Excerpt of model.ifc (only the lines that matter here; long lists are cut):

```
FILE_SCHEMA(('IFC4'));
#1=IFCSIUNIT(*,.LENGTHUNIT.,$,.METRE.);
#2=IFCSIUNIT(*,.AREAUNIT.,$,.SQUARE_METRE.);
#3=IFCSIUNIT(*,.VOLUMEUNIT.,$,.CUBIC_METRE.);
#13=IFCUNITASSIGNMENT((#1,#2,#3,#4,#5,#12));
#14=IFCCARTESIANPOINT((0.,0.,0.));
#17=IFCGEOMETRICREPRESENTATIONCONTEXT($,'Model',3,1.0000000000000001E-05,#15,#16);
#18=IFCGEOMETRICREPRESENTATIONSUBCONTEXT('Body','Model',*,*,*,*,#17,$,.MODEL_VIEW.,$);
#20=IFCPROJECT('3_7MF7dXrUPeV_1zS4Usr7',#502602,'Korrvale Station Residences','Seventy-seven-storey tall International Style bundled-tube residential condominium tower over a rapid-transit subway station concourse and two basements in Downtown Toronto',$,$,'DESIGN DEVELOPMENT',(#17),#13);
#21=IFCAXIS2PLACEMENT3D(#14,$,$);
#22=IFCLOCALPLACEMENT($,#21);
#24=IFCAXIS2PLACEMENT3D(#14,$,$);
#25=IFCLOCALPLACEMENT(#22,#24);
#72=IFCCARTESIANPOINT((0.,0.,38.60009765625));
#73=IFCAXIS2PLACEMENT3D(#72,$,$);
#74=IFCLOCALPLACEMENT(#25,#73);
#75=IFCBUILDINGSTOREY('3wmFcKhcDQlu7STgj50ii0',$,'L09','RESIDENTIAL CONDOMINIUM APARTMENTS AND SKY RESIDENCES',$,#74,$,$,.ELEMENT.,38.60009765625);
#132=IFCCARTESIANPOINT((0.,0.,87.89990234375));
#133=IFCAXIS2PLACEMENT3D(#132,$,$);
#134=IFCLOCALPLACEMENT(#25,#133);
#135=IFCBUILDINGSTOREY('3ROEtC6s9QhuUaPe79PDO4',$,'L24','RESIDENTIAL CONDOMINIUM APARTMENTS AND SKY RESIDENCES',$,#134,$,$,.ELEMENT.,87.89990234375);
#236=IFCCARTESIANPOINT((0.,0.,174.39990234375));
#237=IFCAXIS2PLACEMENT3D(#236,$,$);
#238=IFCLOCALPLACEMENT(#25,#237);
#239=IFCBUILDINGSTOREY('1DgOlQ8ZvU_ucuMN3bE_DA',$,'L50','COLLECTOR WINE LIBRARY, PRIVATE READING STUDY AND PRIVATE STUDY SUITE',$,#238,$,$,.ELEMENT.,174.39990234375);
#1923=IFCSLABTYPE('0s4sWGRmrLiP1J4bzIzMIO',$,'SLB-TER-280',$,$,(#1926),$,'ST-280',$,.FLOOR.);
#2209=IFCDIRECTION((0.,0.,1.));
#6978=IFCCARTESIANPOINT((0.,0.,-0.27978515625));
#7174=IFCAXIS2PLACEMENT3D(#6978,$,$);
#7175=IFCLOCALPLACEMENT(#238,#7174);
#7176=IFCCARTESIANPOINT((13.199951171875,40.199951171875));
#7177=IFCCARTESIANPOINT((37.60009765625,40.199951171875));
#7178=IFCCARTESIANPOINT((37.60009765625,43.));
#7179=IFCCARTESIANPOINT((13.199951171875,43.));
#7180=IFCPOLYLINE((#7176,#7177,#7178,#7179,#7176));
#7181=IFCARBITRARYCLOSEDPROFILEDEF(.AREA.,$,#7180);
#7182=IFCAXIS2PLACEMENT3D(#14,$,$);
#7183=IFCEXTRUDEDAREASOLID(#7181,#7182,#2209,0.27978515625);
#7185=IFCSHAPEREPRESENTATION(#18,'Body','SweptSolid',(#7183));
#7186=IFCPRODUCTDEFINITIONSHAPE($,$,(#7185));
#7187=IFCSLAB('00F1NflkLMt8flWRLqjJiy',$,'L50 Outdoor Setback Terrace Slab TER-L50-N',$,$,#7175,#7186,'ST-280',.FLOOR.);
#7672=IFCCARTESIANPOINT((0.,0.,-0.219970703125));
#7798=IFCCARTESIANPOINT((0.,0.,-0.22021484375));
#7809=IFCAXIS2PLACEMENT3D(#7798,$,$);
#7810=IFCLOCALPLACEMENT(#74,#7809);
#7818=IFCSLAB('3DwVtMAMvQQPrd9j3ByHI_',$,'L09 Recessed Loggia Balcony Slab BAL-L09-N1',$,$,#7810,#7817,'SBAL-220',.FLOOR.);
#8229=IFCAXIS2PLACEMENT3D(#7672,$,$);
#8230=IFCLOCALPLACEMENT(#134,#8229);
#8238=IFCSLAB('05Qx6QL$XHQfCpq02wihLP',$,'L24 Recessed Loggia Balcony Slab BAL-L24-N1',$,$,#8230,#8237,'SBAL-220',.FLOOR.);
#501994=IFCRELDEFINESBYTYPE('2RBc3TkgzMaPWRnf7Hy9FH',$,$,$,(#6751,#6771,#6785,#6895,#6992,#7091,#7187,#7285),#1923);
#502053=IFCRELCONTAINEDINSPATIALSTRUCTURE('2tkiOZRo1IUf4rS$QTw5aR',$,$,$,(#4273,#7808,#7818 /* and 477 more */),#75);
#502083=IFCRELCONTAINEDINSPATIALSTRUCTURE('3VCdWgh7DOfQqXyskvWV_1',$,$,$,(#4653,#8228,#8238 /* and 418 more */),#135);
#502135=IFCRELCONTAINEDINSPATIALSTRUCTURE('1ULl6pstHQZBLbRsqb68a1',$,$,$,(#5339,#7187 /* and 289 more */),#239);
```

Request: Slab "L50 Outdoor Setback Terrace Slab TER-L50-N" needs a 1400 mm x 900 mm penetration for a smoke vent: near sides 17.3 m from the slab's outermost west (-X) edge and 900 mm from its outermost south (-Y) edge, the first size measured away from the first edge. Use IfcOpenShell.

```python
import numpy as np
import ifcopenshell
import ifcopenshell.api.feature
import ifcopenshell.api.geometry
import ifcopenshell.api.root
import ifcopenshell.geom
import ifcopenshell.util.placement
import ifcopenshell.util.representation
import ifcopenshell.util.shape
import ifcopenshell.util.unit

model = ifcopenshell.open("model.ifc")
unit_scale = ifcopenshell.util.unit.calculate_unit_scale(model)
settings = ifcopenshell.geom.settings()


def volume(element):
    """Net volume in cubic metres, openings subtracted."""
    shape = ifcopenshell.geom.create_shape(settings, element)
    return ifcopenshell.util.shape.get_volume(shape.geometry)


slab = model.by_guid("00F1NflkLMt8flWRLqjJiy")
before = volume(slab)

# Extent in the slab's own axes, in metres. The edges named are its -X and -Y sides.
slab_shape = ifcopenshell.geom.create_shape(settings, slab)
vertices = ifcopenshell.util.shape.get_vertices(slab_shape.geometry)
x_min, y_min, bottom = vertices.min(axis=0)
top = vertices[:, 2].max()

opening = ifcopenshell.api.root.create_entity(model, ifc_class="IfcOpeningElement", name="Smoke vent opening", predefined_type="OPENING")
context = ifcopenshell.util.representation.get_context(model, "Model", "Body", "MODEL_VIEW")
width, depth = 1.4, 0.9
outline = [(0.0, 0.0), (width, 0.0), (width, depth), (0.0, depth), (0.0, 0.0)]
# Overshoot both faces by 50 mm so the cut is clean.
shape = ifcopenshell.api.geometry.add_slab_representation(
    model, context=context, depth=top - bottom + 0.1, polyline=outline
)
ifcopenshell.api.geometry.assign_representation(model, product=opening, representation=shape)

matrix = ifcopenshell.util.placement.get_local_placement(slab.ObjectPlacement)
matrix[:, 3] = matrix @ np.append(np.array([x_min + 17.3, y_min + 0.9, bottom - 0.05]) / unit_scale, 1.0)
ifcopenshell.api.geometry.edit_object_placement(model, product=opening, matrix=matrix, is_si=False)
ifcopenshell.api.feature.add_feature(model, feature=opening, element=slab)

after = volume(slab)

print(f"slab volume {before:.3f} -> {after:.3f} m3")

model.write("model_v2.ifc")
```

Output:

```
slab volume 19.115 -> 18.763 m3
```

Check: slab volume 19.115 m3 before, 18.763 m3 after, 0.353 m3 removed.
